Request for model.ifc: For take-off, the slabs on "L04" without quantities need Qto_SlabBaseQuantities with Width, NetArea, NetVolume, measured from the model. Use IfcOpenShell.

First a look at what the model holds.

```python
import ifcopenshell
import ifcopenshell.util.element
import ifcopenshell.util.unit

model = ifcopenshell.open("model.ifc")
print(model.schema)
for unit_type in ("LENGTHUNIT", "AREAUNIT", "VOLUMEUNIT"):
    print(unit_type, ifcopenshell.util.unit.calculate_unit_scale(model, unit_type))
storey = next(s for s in model.by_type("IfcBuildingStorey") if s.Name == "L04")
slabs = [e for e in ifcopenshell.util.element.get_decomposition(storey) if e.is_a("IfcSlab")]
for e in sorted(slabs, key=lambda e: e.id()):
    print(e.id(), e.is_a(), e.Name, list(ifcopenshell.util.element.get_psets(e, qtos_only=True)), sep=" | ")
```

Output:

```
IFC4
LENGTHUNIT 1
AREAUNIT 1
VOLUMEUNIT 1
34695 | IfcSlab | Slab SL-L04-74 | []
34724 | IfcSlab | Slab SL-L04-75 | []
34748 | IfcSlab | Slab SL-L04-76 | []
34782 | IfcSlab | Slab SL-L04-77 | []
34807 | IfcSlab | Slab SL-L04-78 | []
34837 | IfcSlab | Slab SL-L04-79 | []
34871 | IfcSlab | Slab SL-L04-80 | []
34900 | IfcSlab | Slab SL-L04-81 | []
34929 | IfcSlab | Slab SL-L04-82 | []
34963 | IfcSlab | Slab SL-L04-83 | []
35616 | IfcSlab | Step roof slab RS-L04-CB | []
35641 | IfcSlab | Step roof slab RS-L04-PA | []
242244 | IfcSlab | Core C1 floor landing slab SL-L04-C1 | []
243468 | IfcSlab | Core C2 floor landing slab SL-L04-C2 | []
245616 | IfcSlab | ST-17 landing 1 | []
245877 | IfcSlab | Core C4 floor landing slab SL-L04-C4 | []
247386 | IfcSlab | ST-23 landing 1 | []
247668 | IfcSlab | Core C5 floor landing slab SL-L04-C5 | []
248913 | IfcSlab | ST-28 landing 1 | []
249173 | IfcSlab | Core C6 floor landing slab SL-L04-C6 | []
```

```python
import ifcopenshell
import ifcopenshell.api.pset
import ifcopenshell.geom
import ifcopenshell.util.element
import ifcopenshell.util.shape
import ifcopenshell.util.unit

model = ifcopenshell.open("model.ifc")
unit_scale = ifcopenshell.util.unit.calculate_unit_scale(model)
area_scale = ifcopenshell.util.unit.calculate_unit_scale(model, "AREAUNIT")
volume_scale = ifcopenshell.util.unit.calculate_unit_scale(model, "VOLUMEUNIT")
settings = ifcopenshell.geom.settings()

storey = next(s for s in model.by_type("IfcBuildingStorey") if s.Name == "L04")
slabs = [e for e in ifcopenshell.util.element.get_decomposition(storey) if e.is_a("IfcSlab")]

for e in sorted(slabs, key=lambda e: e.id()):
    if ifcopenshell.util.element.get_psets(e, qtos_only=True, should_inherit=False):
        continue
    # Geometry comes back in metres, in the element's own axes.
    shape = ifcopenshell.geom.create_shape(settings, e)
    values = {
        "Width": ifcopenshell.util.shape.get_z(shape.geometry) / unit_scale,
        "NetArea": ifcopenshell.util.shape.get_footprint_area(shape.geometry) / area_scale,
        "NetVolume": ifcopenshell.util.shape.get_volume(shape.geometry) / volume_scale,
    }
    qto = ifcopenshell.api.pset.add_qto(model, product=e, name="Qto_SlabBaseQuantities")
    ifcopenshell.api.pset.edit_qto(model, qto=qto, properties=values)
    print(e.id(), {k: round(v, 3) for k, v in values.items()})

model.write("model_v2.ifc")
```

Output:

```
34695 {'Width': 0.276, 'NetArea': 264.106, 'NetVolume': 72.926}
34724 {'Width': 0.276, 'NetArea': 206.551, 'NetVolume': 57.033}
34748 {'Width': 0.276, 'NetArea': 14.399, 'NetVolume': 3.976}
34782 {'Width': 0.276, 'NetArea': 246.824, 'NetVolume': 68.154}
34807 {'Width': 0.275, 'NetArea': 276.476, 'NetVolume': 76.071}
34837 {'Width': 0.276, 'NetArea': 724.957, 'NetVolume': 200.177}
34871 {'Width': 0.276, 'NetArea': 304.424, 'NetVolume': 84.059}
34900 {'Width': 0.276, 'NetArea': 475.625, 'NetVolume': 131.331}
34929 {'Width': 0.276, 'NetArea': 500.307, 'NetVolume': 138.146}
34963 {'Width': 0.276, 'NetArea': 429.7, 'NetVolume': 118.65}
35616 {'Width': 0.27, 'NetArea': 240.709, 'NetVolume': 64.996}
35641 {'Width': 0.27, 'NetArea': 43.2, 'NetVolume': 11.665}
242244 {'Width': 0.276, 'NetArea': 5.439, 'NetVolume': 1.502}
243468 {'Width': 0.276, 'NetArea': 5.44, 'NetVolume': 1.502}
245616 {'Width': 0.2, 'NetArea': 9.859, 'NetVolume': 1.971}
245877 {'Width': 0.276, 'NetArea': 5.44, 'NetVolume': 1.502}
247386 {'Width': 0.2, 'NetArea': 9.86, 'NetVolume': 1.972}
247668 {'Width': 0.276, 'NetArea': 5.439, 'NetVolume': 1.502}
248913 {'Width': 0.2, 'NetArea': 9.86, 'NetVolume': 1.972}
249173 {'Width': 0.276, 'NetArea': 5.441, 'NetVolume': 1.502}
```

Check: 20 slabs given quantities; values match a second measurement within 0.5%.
